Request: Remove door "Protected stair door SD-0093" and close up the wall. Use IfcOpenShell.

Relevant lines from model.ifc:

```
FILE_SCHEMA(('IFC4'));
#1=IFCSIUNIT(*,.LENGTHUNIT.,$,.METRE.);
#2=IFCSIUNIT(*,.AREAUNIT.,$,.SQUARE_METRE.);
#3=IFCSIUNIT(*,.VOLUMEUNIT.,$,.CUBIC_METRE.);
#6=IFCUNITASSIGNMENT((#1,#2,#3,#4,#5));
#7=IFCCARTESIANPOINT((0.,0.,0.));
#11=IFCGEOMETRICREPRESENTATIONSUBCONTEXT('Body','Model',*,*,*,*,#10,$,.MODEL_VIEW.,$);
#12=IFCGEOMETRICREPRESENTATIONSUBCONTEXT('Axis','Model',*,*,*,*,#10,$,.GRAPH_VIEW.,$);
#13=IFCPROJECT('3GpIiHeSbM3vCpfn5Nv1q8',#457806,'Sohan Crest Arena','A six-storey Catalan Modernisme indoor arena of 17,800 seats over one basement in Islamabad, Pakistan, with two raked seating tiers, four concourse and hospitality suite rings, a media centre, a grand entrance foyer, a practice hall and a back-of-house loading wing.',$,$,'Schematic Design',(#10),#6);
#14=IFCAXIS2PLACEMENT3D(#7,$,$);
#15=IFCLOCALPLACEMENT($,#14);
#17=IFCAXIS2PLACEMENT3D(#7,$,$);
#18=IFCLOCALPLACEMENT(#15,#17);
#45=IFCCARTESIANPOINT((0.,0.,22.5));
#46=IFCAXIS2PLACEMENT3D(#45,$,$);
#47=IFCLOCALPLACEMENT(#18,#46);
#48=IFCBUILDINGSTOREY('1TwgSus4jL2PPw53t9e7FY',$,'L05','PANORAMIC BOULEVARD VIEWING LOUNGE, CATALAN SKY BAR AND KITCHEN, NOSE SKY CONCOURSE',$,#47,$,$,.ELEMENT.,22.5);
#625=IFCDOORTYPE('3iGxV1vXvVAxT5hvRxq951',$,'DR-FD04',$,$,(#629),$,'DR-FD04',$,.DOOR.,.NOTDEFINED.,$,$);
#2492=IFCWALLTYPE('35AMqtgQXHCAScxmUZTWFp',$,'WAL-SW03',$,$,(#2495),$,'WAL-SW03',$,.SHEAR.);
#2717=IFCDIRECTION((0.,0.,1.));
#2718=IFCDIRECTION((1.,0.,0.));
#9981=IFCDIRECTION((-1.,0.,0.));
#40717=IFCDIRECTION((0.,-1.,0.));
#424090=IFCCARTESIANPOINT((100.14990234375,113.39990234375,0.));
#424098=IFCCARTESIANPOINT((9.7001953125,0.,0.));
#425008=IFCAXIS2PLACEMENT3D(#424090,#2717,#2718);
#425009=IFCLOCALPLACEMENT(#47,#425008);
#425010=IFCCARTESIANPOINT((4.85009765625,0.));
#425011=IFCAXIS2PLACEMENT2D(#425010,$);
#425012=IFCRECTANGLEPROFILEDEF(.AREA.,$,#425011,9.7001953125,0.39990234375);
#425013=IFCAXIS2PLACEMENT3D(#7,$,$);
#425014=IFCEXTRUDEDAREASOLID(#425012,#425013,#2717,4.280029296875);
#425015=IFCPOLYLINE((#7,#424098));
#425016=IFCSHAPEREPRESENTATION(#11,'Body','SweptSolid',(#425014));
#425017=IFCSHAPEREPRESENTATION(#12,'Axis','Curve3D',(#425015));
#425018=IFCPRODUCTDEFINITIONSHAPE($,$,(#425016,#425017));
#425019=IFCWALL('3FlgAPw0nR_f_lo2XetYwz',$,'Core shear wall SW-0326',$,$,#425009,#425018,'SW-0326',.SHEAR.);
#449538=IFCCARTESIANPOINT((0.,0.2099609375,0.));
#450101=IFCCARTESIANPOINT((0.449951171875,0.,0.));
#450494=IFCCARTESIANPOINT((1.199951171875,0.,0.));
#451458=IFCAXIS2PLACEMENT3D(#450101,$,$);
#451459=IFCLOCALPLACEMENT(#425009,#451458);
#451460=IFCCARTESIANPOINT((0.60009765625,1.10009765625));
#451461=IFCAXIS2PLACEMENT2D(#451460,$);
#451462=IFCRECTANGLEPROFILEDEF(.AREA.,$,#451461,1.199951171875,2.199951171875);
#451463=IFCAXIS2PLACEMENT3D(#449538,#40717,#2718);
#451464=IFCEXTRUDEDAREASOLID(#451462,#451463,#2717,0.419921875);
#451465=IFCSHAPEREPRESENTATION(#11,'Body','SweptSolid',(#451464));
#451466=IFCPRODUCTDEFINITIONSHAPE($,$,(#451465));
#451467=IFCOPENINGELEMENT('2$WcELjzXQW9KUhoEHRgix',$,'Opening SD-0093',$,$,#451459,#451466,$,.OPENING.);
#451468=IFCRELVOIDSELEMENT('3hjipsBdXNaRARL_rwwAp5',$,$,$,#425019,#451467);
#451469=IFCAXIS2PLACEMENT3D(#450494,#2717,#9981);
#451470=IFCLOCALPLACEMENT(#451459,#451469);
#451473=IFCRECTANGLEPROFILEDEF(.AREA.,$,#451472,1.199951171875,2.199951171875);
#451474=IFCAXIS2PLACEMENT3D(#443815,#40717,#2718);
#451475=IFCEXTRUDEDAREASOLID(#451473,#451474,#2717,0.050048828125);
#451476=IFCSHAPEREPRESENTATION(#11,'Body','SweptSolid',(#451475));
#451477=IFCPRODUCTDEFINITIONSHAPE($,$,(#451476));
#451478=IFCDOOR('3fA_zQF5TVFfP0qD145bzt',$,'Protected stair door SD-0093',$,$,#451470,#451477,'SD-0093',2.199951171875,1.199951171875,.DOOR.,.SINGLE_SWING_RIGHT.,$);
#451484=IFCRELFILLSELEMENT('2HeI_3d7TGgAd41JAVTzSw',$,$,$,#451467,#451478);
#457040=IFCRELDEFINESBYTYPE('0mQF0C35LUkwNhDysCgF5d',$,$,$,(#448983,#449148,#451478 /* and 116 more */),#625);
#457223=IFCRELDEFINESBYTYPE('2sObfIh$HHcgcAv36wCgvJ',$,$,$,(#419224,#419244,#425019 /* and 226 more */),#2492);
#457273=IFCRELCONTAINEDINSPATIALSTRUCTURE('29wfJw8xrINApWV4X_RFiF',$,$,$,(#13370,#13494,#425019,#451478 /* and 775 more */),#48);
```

```python
import ifcopenshell
import ifcopenshell.api.feature
import ifcopenshell.api.root
import ifcopenshell.geom
import ifcopenshell.util.shape

model = ifcopenshell.open("model.ifc")
settings = ifcopenshell.geom.settings()


def volume(element):
    """Net volume in cubic metres, openings subtracted."""
    shape = ifcopenshell.geom.create_shape(settings, element)
    return ifcopenshell.util.shape.get_volume(shape.geometry)


door = model.by_guid("3fA_zQF5TVFfP0qD145bzt")
opening = door.FillsVoids[0].RelatingOpeningElement
wall = opening.VoidsElements[0].RelatingBuildingElement
before = volume(wall)

ifcopenshell.api.root.remove_product(model, product=door)
ifcopenshell.api.feature.remove_feature(model, feature=opening)

after = volume(wall)

print(f"wall volume {before:.3f} -> {after:.3f} m3")

model.write("model_updated.ifc")
```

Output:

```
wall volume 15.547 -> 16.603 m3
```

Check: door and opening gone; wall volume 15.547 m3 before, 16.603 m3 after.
